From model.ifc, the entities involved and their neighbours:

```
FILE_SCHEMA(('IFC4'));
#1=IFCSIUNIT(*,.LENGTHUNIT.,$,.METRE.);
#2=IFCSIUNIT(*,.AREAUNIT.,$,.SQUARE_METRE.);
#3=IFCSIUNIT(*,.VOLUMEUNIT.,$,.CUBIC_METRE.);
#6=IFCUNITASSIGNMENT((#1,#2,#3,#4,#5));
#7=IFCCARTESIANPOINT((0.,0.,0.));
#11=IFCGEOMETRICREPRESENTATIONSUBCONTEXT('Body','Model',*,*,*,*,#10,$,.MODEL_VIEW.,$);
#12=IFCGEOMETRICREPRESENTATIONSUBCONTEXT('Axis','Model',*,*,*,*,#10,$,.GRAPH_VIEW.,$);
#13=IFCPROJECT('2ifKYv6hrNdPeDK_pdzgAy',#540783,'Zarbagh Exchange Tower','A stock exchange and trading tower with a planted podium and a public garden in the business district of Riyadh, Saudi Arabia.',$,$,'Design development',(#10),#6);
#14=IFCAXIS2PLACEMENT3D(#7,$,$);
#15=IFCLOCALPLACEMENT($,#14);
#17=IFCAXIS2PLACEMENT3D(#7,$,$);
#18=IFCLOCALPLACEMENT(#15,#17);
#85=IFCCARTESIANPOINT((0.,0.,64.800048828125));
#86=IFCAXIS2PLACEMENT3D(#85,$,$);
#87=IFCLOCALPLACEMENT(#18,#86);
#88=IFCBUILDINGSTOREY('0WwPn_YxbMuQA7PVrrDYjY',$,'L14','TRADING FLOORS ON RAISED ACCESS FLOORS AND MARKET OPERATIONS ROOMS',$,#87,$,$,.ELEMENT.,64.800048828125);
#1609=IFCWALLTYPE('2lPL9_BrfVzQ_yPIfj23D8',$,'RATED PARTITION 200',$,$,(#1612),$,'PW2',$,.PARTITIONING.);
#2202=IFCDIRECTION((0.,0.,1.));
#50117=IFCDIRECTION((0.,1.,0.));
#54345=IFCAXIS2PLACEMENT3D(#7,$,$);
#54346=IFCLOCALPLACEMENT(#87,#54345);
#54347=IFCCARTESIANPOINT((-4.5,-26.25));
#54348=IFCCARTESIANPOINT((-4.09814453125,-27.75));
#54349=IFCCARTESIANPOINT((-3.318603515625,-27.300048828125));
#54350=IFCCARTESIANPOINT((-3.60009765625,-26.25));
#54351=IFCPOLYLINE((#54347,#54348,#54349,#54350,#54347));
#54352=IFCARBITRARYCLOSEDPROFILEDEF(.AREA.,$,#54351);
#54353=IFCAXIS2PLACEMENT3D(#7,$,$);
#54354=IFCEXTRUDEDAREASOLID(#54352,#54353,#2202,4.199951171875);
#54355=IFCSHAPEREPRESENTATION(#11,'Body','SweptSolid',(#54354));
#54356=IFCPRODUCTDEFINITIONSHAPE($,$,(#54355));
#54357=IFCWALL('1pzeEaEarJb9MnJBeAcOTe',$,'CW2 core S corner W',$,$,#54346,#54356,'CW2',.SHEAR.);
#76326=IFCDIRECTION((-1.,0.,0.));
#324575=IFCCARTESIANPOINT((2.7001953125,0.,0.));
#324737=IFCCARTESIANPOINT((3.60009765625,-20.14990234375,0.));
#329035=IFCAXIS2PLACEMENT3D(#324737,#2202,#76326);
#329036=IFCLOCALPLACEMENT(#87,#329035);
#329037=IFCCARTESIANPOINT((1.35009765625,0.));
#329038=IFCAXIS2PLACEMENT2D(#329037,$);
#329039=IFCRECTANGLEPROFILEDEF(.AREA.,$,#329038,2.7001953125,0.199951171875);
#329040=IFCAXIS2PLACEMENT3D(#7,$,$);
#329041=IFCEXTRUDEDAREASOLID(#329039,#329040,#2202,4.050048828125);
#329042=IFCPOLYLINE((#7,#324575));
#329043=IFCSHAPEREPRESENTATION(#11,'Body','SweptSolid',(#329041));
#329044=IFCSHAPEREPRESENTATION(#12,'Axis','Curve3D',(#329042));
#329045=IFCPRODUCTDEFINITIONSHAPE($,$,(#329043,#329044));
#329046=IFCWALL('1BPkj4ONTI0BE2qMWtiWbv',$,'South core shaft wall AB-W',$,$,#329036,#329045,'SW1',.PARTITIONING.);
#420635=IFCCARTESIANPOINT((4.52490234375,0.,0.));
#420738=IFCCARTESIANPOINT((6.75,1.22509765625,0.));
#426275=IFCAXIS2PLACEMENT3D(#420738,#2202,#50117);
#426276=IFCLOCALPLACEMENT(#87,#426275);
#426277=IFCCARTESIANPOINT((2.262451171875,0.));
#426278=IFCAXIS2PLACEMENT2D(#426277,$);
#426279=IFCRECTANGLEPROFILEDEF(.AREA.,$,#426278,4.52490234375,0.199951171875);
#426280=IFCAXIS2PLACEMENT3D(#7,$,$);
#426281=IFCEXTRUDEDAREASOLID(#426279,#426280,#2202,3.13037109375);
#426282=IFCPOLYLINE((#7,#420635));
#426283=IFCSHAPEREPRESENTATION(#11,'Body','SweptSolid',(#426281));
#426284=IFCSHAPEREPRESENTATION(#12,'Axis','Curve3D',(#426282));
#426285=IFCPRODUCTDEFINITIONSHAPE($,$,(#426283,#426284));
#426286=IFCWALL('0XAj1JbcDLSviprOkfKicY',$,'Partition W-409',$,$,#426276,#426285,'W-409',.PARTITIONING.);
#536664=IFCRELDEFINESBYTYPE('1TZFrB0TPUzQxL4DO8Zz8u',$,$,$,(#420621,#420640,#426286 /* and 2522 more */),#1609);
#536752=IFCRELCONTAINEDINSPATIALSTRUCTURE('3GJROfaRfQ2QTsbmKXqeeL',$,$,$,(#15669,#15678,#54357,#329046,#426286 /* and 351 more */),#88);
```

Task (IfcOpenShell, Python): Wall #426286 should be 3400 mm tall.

```python
import ifcopenshell
import ifcopenshell.geom
import ifcopenshell.util.representation
import ifcopenshell.util.shape

model = ifcopenshell.open("model.ifc")
settings = ifcopenshell.geom.settings()


def volume(element):
    """Net volume in cubic metres, openings subtracted."""
    shape = ifcopenshell.geom.create_shape(settings, element)
    return ifcopenshell.util.shape.get_volume(shape.geometry)


wall = model.by_guid("0XAj1JbcDLSviprOkfKicY")
before = volume(wall)

body = ifcopenshell.util.representation.get_representation(wall, "Model", "Body")
solid = body.Items[0]
old_height = solid.Depth
solid.Depth = 3.4
after = volume(wall)

print(f"height {old_height:g} -> {solid.Depth:g}, volume {before:.3f} -> {after:.3f} m3")

model.write("model_rev.ifc")
```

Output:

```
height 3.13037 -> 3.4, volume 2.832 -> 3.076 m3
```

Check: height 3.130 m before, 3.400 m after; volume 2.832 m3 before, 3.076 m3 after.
